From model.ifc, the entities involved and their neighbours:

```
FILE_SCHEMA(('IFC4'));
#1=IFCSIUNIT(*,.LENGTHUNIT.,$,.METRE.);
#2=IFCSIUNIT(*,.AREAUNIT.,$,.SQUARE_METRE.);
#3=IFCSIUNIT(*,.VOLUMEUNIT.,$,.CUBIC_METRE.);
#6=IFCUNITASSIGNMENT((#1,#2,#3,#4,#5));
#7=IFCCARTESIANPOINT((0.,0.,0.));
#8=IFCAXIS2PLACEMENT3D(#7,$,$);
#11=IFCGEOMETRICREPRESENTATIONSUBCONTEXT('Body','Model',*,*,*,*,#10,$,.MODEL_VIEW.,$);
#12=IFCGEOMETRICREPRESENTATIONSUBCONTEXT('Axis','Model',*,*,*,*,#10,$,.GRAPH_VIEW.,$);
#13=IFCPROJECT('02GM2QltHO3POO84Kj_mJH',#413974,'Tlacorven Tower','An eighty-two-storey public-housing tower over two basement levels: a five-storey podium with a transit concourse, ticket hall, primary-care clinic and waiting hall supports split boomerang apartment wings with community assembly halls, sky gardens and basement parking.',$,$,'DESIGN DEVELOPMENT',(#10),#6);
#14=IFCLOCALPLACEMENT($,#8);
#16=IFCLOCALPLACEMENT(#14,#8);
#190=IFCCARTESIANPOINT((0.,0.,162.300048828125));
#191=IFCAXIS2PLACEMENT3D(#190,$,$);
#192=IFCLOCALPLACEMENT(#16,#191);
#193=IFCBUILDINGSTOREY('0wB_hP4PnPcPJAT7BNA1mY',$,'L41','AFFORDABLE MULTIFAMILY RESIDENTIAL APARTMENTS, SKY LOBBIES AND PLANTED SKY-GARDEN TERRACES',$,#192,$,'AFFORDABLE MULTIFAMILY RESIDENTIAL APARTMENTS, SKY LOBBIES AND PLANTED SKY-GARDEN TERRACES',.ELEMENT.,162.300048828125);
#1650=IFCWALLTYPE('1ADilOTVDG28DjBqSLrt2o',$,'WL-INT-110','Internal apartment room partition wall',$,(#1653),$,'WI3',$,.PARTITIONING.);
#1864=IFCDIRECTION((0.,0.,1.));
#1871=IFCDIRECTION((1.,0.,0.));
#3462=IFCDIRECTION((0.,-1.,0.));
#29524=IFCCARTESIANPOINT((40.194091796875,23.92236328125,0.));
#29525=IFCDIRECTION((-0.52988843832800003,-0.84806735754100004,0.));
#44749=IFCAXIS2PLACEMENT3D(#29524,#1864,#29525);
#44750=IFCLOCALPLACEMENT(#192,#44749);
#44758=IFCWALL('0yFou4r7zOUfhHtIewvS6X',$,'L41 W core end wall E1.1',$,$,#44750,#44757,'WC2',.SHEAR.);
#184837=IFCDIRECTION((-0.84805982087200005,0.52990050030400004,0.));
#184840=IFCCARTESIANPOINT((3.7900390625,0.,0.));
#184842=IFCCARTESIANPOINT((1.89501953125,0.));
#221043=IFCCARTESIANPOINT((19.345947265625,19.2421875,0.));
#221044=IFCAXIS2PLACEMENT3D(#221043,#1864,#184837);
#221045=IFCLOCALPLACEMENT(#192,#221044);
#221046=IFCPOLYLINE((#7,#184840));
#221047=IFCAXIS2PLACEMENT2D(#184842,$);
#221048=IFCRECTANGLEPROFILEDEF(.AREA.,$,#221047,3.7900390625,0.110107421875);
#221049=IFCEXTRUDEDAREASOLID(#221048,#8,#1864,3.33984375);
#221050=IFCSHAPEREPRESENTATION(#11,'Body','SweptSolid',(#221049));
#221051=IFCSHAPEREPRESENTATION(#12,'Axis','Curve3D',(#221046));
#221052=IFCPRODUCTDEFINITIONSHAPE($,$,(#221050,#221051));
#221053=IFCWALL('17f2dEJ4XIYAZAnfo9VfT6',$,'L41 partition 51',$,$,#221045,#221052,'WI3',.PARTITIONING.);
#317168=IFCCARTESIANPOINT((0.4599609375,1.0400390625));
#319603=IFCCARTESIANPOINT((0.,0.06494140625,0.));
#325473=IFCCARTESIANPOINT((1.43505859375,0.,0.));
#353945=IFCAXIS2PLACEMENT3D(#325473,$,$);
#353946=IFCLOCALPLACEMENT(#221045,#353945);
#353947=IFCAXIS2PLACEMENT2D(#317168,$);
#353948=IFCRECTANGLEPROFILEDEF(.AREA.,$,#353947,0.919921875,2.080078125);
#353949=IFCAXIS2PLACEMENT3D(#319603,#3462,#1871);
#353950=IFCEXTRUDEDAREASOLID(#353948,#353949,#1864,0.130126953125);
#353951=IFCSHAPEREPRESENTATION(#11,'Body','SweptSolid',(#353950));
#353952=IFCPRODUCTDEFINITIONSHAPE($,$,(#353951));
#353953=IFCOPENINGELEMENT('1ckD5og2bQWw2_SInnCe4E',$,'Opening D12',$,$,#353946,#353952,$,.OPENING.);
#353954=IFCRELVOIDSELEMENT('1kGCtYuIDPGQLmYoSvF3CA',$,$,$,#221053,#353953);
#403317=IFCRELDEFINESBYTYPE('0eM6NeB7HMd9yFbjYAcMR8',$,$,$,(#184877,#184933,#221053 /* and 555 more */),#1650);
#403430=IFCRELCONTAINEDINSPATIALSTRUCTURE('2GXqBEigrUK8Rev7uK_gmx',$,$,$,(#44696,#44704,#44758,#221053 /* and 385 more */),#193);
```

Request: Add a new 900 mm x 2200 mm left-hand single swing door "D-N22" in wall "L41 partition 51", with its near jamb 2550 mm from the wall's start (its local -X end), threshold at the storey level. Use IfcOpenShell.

```python
import numpy as np
import ifcopenshell
import ifcopenshell.api.feature
import ifcopenshell.api.geometry
import ifcopenshell.api.root
import ifcopenshell.api.spatial
import ifcopenshell.geom
import ifcopenshell.util.element
import ifcopenshell.util.placement
import ifcopenshell.util.representation
import ifcopenshell.util.shape
import ifcopenshell.util.unit

model = ifcopenshell.open("model.ifc")
unit_scale = ifcopenshell.util.unit.calculate_unit_scale(model)
settings = ifcopenshell.geom.settings()


def volume(element):
    """Net volume in cubic metres, openings subtracted."""
    shape = ifcopenshell.geom.create_shape(settings, element)
    return ifcopenshell.util.shape.get_volume(shape.geometry)


wall = model.by_guid("17f2dEJ4XIYAZAnfo9VfT6")
storey = ifcopenshell.util.element.get_container(wall, ifc_class="IfcBuildingStorey")
context = ifcopenshell.util.representation.get_context(model, "Model", "Body", "MODEL_VIEW")
before = volume(wall)

width, height, from_end, sill = 0.9, 2.2, 2.55, 0.0  # metres

# The wall runs along its own X axis, and the end named is its -X end.
wall_shape = ifcopenshell.geom.create_shape(settings, wall)
x, y, z = ifcopenshell.util.shape.get_vertices(wall_shape.geometry).T
start = x.min() + from_end
face, thickness = float(y.min()), float(y.max() - y.min())
wall_matrix = ifcopenshell.util.placement.get_local_placement(wall.ObjectPlacement)
level = ifcopenshell.util.placement.get_local_placement(storey.ObjectPlacement)[2, 3]


def in_wall(x, y):
    """Placement at x, y metres in the wall's axes, at sill height."""
    matrix = wall_matrix.copy()
    matrix[:, 3] = wall_matrix @ np.array([x / unit_scale, y / unit_scale, 0.0, 1.0])
    matrix[2, 3] = level + sill / unit_scale
    return matrix


# Opening: a box that overshoots both wall faces by 50 mm.
opening = ifcopenshell.api.root.create_entity(model, ifc_class="IfcOpeningElement", predefined_type="OPENING")
box = ifcopenshell.api.geometry.add_wall_representation(
    model, context=context, length=width, height=height, thickness=thickness + 0.1
)
ifcopenshell.api.geometry.assign_representation(model, product=opening, representation=box)
ifcopenshell.api.geometry.edit_object_placement(model, product=opening, matrix=in_wall(start, face - 0.05), is_si=False)
ifcopenshell.api.feature.add_feature(model, feature=opening, element=wall)

door = ifcopenshell.api.root.create_entity(model, ifc_class="IfcDoor", name="D-N22", predefined_type="DOOR")
door.OverallWidth, door.OverallHeight = width / unit_scale, height / unit_scale
door.OperationType = "SINGLE_SWING_LEFT"
body = ifcopenshell.api.geometry.add_door_representation(
    model,
    context=context,
    overall_width=door.OverallWidth,
    overall_height=door.OverallHeight,
    operation_type="SINGLE_SWING_LEFT",
    lining_properties={"LiningDepth": thickness / unit_scale, "ThresholdDepth": thickness / unit_scale},
)
ifcopenshell.api.geometry.assign_representation(model, product=door, representation=body)
ifcopenshell.api.spatial.assign_container(model, products=[door], relating_structure=storey)
ifcopenshell.api.feature.add_filling(model, opening=opening, element=door)

# The lining spans the wall, so the door starts at the wall face.
ifcopenshell.api.geometry.edit_object_placement(model, product=door, matrix=in_wall(start, face), is_si=False)

after = volume(wall)

print(f"wall volume {before:.3f} -> {after:.3f} m3")

model.write("model_edited.ifc")
```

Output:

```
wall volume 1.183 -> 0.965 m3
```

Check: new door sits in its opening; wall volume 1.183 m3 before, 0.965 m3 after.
